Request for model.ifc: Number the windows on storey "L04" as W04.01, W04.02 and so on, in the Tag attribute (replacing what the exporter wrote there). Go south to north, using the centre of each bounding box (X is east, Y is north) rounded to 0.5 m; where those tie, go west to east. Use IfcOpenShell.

First a look at what the model holds.

```python
import ifcopenshell
import ifcopenshell.util.element
import ifcopenshell.util.placement

model = ifcopenshell.open("model.ifc")
print(model.schema)
storey = next(s for s in model.by_type("IfcBuildingStorey") if s.Name == "L04")
windows = [e for e in ifcopenshell.util.element.get_decomposition(storey) if e.is_a("IfcWindow")]
for e in sorted(windows, key=lambda e: e.id()):
    origin = ifcopenshell.util.placement.get_local_placement(e.ObjectPlacement)[:3, 3]
    print(e.id(), e.Tag, e.Name, origin.round(2) + 0.0, sep=" | ")
```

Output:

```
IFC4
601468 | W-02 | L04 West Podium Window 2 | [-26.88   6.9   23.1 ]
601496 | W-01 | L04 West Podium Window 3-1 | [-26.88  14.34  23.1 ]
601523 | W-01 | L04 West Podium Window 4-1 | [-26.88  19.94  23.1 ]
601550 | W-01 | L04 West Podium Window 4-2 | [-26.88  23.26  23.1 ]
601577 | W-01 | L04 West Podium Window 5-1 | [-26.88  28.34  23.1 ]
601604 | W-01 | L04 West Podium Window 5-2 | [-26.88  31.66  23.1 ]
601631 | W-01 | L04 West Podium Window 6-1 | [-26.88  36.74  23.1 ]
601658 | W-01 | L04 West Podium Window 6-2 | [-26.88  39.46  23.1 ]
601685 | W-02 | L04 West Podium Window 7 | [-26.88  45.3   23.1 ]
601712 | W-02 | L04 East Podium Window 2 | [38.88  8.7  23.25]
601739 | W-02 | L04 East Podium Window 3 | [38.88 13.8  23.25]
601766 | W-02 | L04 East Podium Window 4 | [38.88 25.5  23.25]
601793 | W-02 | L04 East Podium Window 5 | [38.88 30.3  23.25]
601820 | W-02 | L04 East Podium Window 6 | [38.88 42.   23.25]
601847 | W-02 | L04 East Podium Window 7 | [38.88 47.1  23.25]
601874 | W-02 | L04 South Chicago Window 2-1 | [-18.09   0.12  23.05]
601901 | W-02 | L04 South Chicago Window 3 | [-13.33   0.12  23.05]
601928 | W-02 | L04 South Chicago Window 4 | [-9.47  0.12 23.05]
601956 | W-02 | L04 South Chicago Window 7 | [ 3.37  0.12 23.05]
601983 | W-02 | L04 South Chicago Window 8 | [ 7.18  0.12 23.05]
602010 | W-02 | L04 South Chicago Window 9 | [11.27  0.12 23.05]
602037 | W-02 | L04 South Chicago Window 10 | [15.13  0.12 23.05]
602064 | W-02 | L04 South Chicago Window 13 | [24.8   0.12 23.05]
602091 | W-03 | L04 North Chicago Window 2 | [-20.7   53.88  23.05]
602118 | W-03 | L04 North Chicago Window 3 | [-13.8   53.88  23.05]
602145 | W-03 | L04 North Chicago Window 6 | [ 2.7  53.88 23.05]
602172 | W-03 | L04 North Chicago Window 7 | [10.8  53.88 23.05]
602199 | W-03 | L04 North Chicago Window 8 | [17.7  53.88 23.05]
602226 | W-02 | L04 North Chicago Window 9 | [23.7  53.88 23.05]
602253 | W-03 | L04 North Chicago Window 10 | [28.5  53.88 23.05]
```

```python
import ifcopenshell
import ifcopenshell.geom
import ifcopenshell.util.element
import ifcopenshell.util.shape

model = ifcopenshell.open("model.ifc")
settings = ifcopenshell.geom.settings()
settings.set("use-world-coords", True)


def centre(element):
    shape = ifcopenshell.geom.create_shape(settings, element)
    return ifcopenshell.util.shape.get_bbox_centroid(shape.geometry)


storey = next(s for s in model.by_type("IfcBuildingStorey") if s.Name == "L04")
windows = [e for e in ifcopenshell.util.element.get_decomposition(storey) if e.is_a("IfcWindow")]

# Insertion points can sit at a corner or the storey origin, so sort by the geometry (in metres).
centres = {e: centre(e) for e in windows}
windows.sort(key=lambda e: (round(centres[e][1] / 0.5), centres[e][0]))

for i, e in enumerate(windows, start=1):
    number = f"W04.{i:02d}"
    e.Tag = number
    print(e.id(), number)

model.write("model_updated.ifc")
```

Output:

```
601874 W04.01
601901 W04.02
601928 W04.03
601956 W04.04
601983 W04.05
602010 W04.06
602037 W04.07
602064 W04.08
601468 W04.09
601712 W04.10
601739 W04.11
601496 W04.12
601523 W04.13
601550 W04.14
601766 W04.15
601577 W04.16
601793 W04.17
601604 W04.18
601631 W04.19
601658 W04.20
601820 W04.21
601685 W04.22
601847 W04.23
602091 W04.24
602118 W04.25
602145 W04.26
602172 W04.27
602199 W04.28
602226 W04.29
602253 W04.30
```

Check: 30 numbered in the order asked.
